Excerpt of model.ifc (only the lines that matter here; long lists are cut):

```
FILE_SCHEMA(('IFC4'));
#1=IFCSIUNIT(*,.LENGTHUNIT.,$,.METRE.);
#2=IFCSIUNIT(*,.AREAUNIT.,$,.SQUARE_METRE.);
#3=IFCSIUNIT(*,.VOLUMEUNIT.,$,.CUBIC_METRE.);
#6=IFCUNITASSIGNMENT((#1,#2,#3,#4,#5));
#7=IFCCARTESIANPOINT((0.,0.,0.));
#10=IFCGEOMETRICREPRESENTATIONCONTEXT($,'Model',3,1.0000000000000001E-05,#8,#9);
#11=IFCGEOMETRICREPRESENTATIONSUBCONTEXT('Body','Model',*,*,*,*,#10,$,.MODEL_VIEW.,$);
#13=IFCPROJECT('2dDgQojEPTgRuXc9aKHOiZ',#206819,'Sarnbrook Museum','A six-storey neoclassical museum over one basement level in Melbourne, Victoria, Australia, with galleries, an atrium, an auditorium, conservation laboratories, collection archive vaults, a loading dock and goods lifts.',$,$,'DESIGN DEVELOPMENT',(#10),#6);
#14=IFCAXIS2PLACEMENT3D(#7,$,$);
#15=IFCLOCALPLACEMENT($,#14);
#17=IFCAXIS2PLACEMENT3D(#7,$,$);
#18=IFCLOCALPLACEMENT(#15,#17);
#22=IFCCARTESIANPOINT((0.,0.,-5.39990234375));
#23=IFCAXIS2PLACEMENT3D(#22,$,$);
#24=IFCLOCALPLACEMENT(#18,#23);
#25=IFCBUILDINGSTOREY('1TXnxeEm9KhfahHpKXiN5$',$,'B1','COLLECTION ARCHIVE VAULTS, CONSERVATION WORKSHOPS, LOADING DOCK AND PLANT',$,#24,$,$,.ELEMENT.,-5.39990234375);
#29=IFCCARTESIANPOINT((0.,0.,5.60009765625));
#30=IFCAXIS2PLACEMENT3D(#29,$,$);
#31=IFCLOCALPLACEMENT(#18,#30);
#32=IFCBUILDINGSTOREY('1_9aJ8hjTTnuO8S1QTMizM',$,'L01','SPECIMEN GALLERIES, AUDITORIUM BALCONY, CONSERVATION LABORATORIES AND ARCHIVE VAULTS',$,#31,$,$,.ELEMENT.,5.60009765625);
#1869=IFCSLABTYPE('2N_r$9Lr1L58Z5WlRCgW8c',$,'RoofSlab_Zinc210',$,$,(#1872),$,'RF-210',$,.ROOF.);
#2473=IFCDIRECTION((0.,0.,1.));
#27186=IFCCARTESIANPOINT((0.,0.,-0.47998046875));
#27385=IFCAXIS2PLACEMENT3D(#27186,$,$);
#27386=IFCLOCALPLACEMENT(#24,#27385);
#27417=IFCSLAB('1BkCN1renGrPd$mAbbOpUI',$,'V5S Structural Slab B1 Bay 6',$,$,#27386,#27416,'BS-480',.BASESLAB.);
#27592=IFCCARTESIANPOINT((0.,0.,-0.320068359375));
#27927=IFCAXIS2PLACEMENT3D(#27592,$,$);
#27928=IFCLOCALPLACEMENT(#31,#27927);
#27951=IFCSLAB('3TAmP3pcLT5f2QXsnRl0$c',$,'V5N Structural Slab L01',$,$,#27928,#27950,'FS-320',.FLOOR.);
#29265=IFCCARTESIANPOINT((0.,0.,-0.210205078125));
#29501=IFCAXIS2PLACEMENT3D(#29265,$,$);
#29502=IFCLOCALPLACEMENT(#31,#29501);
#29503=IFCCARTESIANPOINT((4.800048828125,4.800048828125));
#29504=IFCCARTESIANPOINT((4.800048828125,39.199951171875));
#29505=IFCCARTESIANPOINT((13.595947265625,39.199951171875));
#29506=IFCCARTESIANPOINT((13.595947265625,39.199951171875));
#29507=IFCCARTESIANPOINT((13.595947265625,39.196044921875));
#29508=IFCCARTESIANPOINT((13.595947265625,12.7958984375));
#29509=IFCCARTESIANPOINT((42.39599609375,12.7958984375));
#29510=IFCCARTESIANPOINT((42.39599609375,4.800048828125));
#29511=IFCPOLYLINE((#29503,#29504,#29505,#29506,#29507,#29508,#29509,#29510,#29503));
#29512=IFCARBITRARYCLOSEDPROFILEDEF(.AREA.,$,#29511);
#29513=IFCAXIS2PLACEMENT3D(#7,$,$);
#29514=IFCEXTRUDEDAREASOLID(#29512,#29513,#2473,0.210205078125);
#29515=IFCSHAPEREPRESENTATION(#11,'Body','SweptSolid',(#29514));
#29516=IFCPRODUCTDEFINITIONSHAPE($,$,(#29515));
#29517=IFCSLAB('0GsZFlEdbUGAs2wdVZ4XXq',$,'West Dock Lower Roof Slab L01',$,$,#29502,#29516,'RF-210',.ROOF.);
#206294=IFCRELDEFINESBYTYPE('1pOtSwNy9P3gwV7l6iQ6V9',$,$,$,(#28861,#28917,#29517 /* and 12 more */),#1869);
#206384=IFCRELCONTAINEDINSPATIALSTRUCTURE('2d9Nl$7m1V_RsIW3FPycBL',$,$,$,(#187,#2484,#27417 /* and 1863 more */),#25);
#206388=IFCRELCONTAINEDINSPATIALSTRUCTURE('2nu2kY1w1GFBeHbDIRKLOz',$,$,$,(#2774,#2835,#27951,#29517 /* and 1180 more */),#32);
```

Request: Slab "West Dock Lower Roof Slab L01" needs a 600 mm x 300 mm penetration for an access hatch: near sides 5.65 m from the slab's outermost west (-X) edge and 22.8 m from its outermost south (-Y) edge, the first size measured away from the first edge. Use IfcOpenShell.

```python
import numpy as np
import ifcopenshell
import ifcopenshell.api.feature
import ifcopenshell.api.geometry
import ifcopenshell.api.root
import ifcopenshell.geom
import ifcopenshell.util.placement
import ifcopenshell.util.representation
import ifcopenshell.util.shape
import ifcopenshell.util.unit

model = ifcopenshell.open("model.ifc")
unit_scale = ifcopenshell.util.unit.calculate_unit_scale(model)
settings = ifcopenshell.geom.settings()


def volume(element):
    """Net volume in cubic metres, openings subtracted."""
    shape = ifcopenshell.geom.create_shape(settings, element)
    return ifcopenshell.util.shape.get_volume(shape.geometry)


slab = model.by_guid("0GsZFlEdbUGAs2wdVZ4XXq")
before = volume(slab)

# Extent in the slab's own axes, in metres. The edges named are its -X and -Y sides.
slab_shape = ifcopenshell.geom.create_shape(settings, slab)
vertices = ifcopenshell.util.shape.get_vertices(slab_shape.geometry)
x_min, y_min, bottom = vertices.min(axis=0)
top = vertices[:, 2].max()

opening = ifcopenshell.api.root.create_entity(model, ifc_class="IfcOpeningElement", name="Access hatch opening", predefined_type="OPENING")
context = ifcopenshell.util.representation.get_context(model, "Model", "Body", "MODEL_VIEW")
width, depth = 0.6, 0.3
outline = [(0.0, 0.0), (width, 0.0), (width, depth), (0.0, depth), (0.0, 0.0)]
# Overshoot both faces by 50 mm so the cut is clean.
shape = ifcopenshell.api.geometry.add_slab_representation(
    model, context=context, depth=top - bottom + 0.1, polyline=outline
)
ifcopenshell.api.geometry.assign_representation(model, product=opening, representation=shape)

matrix = ifcopenshell.util.placement.get_local_placement(slab.ObjectPlacement)
matrix[:, 3] = matrix @ np.append(np.array([x_min + 5.65, y_min + 22.8, bottom - 0.05]) / unit_scale, 1.0)
ifcopenshell.api.geometry.edit_object_placement(model, product=opening, matrix=matrix, is_si=False)
ifcopenshell.api.feature.add_feature(model, feature=opening, element=slab)

after = volume(slab)

print(f"slab volume {before:.3f} -> {after:.3f} m3")

model.write("model_updated.ifc")
```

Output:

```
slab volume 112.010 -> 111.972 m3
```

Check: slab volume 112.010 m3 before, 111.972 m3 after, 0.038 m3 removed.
